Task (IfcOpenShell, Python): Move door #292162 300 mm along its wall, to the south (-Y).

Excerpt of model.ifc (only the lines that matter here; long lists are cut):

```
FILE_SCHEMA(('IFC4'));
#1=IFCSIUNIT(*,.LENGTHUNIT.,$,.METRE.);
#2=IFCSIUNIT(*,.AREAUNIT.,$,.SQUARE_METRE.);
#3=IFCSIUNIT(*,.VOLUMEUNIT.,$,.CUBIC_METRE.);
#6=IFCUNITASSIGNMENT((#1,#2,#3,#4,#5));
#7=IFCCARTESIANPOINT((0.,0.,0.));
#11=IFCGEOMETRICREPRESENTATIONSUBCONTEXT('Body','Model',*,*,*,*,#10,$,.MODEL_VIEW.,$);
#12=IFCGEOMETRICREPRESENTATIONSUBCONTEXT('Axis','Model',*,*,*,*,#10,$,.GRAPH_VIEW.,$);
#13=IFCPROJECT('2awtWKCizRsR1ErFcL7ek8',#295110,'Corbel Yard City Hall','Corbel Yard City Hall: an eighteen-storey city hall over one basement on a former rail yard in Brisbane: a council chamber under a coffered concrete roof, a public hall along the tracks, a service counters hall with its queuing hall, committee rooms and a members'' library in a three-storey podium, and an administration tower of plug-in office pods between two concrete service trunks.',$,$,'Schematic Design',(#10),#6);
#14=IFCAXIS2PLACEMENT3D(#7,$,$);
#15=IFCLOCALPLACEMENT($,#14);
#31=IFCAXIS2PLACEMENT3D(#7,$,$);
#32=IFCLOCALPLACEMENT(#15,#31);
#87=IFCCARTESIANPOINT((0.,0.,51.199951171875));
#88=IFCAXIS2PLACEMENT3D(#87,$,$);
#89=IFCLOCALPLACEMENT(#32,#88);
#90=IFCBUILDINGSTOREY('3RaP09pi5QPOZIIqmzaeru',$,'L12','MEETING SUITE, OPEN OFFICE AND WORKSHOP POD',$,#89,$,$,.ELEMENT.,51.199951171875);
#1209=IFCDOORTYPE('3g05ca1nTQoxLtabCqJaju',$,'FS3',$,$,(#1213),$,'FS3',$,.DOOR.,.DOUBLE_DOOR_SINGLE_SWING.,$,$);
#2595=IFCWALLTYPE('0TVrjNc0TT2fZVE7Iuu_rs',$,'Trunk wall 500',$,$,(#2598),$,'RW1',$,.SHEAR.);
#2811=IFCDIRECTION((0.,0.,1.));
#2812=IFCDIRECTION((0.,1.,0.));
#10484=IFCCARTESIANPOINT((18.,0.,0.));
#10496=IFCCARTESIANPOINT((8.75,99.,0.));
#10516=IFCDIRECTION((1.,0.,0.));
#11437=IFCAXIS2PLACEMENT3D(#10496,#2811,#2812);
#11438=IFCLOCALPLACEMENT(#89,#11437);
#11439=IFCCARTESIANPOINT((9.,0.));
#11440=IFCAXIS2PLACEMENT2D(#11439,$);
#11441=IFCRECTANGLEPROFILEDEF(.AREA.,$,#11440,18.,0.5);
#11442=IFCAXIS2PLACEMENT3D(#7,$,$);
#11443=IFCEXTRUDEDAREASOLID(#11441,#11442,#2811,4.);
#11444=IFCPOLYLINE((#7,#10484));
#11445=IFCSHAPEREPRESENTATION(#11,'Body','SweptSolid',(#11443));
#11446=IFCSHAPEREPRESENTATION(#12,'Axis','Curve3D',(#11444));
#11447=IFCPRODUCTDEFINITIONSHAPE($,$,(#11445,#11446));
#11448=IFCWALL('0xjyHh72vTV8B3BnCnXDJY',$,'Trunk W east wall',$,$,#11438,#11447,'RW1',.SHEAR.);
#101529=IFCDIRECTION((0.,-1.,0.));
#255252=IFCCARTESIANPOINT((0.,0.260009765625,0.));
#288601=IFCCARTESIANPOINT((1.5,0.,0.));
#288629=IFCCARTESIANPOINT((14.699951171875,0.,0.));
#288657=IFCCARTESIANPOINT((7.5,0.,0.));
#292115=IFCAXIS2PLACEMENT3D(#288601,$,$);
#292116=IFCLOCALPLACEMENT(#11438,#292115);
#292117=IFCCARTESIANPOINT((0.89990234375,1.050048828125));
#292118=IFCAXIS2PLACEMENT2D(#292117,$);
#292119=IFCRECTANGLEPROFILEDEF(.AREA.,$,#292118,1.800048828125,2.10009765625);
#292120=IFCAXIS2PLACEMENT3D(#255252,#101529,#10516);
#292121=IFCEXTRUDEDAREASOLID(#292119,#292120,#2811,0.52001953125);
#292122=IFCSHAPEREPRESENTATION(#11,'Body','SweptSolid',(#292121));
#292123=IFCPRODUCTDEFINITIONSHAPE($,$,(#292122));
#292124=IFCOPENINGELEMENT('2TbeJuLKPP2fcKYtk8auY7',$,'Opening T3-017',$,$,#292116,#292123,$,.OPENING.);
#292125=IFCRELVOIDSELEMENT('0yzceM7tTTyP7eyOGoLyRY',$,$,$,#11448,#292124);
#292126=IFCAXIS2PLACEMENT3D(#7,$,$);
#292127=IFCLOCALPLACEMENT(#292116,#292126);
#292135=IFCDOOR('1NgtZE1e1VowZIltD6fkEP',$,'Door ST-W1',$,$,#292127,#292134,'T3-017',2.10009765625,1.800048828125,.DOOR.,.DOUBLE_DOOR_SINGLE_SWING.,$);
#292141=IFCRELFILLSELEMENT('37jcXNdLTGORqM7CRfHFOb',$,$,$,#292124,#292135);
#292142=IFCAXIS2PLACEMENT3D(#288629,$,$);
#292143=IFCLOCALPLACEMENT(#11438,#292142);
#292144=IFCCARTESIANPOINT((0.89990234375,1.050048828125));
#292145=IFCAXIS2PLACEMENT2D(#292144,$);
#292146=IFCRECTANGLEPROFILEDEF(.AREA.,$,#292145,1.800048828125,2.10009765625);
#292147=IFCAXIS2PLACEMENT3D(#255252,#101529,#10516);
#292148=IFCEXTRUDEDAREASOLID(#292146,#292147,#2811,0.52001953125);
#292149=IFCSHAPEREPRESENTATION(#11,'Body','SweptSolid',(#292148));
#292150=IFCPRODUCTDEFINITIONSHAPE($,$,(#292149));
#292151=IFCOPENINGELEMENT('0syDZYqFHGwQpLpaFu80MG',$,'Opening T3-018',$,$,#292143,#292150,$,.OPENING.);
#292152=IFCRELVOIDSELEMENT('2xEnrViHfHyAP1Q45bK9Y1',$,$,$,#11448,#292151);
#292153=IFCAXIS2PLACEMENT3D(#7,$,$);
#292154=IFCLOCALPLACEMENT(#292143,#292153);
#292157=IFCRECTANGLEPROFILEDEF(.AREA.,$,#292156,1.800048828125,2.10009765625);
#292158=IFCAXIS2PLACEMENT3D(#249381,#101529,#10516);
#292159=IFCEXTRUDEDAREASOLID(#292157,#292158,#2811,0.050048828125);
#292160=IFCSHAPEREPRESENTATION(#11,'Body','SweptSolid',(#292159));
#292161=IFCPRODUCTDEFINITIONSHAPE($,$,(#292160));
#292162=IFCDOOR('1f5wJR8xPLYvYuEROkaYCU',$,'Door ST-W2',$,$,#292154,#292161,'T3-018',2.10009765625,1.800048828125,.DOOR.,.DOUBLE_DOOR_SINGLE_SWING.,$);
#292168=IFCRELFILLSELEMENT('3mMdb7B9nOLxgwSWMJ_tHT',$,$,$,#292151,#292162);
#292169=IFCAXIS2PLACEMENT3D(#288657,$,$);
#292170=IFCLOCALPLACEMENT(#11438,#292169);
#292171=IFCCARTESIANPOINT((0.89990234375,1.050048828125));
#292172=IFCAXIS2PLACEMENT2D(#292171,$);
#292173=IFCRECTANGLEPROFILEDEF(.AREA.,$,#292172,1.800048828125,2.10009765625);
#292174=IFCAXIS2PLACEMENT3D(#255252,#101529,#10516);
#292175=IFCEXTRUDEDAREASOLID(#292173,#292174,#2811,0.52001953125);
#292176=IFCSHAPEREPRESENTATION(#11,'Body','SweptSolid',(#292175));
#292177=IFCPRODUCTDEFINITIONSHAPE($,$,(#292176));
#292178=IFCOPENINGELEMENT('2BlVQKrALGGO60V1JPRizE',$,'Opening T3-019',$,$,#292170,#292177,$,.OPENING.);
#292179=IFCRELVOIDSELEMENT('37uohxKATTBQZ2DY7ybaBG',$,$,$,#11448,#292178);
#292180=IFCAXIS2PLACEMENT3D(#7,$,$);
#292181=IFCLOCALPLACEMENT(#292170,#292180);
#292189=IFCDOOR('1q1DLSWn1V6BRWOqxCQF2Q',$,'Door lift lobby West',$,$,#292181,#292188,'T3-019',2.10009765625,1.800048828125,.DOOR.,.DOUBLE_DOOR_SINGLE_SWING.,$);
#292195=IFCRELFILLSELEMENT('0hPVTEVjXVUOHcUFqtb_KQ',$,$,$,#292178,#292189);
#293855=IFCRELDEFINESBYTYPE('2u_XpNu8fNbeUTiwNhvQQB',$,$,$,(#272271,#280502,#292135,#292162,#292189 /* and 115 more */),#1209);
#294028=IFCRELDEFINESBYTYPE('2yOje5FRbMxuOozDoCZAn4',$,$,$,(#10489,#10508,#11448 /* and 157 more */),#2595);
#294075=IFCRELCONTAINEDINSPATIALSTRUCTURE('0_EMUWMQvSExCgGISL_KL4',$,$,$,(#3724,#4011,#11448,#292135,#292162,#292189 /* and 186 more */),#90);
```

```python
import ifcopenshell
import ifcopenshell.api.geometry
import ifcopenshell.util.placement
import ifcopenshell.util.unit

model = ifcopenshell.open("model.ifc")
unit_scale = ifcopenshell.util.unit.calculate_unit_scale(model)

door = model.by_guid("1f5wJR8xPLYvYuEROkaYCU")
opening = door.FillsVoids[0].RelatingOpeningElement
wall = opening.VoidsElements[0].RelatingBuildingElement

wall_matrix = ifcopenshell.util.placement.get_local_placement(wall.ObjectPlacement)
shift = wall_matrix[:3, 0] * -0.3 / unit_scale
before = ifcopenshell.util.placement.get_local_placement(door.ObjectPlacement)[:3, 3].copy()

# The door is placed relative to its opening, so it follows when the opening moves.
matrix = ifcopenshell.util.placement.get_local_placement(opening.ObjectPlacement)
matrix[:3, 3] += shift
ifcopenshell.api.geometry.edit_object_placement(
    model, product=opening, matrix=matrix, is_si=False, should_transform_children=True
)

after = ifcopenshell.util.placement.get_local_placement(door.ObjectPlacement)[:3, 3]
print("door moved by", (after - before).round(3) + 0.0)

model.write("model_edited.ifc")
```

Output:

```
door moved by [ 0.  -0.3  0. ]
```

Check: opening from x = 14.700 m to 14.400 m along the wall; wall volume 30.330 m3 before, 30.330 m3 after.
